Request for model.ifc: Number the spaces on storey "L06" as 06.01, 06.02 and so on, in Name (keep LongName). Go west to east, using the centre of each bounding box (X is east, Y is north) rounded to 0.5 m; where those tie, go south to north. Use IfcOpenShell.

First a look at what the model holds.

```python
import ifcopenshell
import ifcopenshell.util.element
import ifcopenshell.util.placement

model = ifcopenshell.open("model.ifc")
print(model.schema)
storey = next(s for s in model.by_type("IfcBuildingStorey") if s.Name == "L06")
spaces = [e for e in ifcopenshell.util.element.get_decomposition(storey) if e.is_a("IfcSpace")]
for e in sorted(spaces, key=lambda e: e.id()):
    origin = ifcopenshell.util.placement.get_local_placement(e.ObjectPlacement)[:3, 3]
    print(e.id(), e.Name, e.LongName, origin.round(2) + 0.0, sep=" | ")
```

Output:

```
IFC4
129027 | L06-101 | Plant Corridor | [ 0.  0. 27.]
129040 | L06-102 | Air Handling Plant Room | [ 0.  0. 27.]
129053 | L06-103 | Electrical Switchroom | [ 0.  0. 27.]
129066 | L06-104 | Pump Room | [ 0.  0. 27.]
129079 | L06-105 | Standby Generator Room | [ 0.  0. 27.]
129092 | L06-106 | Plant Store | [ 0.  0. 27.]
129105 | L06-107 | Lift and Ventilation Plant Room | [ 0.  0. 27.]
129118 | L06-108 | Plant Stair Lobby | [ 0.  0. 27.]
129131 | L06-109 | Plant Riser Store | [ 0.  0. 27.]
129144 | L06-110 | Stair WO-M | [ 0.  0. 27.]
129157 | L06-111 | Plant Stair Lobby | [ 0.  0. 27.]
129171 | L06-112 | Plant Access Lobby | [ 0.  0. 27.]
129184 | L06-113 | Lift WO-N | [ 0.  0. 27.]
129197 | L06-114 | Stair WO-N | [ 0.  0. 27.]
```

```python
import ifcopenshell
import ifcopenshell.geom
import ifcopenshell.util.element
import ifcopenshell.util.shape

model = ifcopenshell.open("model.ifc")
settings = ifcopenshell.geom.settings()
settings.set("use-world-coords", True)


def centre(element):
    shape = ifcopenshell.geom.create_shape(settings, element)
    return ifcopenshell.util.shape.get_bbox_centroid(shape.geometry)


storey = next(s for s in model.by_type("IfcBuildingStorey") if s.Name == "L06")
spaces = [e for e in ifcopenshell.util.element.get_decomposition(storey) if e.is_a("IfcSpace")]

# Insertion points can sit at a corner or the storey origin, so sort by the geometry (in metres).
centres = {e: centre(e) for e in spaces}
spaces.sort(key=lambda e: (round(centres[e][0] / 0.5), centres[e][1]))

for i, e in enumerate(spaces, start=1):
    number = f"06.{i:02d}"
    e.Name = number
    print(e.id(), number)

model.write("model-out.ifc")
```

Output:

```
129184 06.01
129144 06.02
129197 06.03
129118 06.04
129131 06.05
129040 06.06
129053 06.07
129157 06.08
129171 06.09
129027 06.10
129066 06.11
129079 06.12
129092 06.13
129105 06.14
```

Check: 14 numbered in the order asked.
